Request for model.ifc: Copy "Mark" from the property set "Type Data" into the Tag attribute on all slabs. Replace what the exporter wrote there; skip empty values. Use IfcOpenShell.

First a look at what the model holds.

```python
import ifcopenshell
import ifcopenshell.util.element

model = ifcopenshell.open("model.ifc")
print(model.schema)
slabs = model.by_type("IfcSlab")
print(len(slabs), "slabs")
for e in slabs[:8]:
    source = ifcopenshell.util.element.get_pset(e, "Type Data", "Mark")
    target = e.Tag
    print(e.id(), repr(source), repr(target), sep=" | ")
```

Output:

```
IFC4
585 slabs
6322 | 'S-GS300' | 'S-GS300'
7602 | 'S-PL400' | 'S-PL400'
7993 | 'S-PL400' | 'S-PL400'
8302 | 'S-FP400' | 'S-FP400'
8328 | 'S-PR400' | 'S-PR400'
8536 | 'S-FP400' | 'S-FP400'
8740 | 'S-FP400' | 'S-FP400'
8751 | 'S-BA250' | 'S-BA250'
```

```python
import ifcopenshell
import ifcopenshell.util.element

model = ifcopenshell.open("model.ifc")

count = 0
for e in model.by_type("IfcSlab"):
    value = ifcopenshell.util.element.get_pset(e, "Type Data", "Mark")
    current = e.Tag
    if not value or not value.strip() or current == value:
        continue
    e.Tag = value
    count += 1

print(count, "slabs updated")

model.write("model_rev.ifc")
```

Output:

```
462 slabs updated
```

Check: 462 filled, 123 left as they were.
